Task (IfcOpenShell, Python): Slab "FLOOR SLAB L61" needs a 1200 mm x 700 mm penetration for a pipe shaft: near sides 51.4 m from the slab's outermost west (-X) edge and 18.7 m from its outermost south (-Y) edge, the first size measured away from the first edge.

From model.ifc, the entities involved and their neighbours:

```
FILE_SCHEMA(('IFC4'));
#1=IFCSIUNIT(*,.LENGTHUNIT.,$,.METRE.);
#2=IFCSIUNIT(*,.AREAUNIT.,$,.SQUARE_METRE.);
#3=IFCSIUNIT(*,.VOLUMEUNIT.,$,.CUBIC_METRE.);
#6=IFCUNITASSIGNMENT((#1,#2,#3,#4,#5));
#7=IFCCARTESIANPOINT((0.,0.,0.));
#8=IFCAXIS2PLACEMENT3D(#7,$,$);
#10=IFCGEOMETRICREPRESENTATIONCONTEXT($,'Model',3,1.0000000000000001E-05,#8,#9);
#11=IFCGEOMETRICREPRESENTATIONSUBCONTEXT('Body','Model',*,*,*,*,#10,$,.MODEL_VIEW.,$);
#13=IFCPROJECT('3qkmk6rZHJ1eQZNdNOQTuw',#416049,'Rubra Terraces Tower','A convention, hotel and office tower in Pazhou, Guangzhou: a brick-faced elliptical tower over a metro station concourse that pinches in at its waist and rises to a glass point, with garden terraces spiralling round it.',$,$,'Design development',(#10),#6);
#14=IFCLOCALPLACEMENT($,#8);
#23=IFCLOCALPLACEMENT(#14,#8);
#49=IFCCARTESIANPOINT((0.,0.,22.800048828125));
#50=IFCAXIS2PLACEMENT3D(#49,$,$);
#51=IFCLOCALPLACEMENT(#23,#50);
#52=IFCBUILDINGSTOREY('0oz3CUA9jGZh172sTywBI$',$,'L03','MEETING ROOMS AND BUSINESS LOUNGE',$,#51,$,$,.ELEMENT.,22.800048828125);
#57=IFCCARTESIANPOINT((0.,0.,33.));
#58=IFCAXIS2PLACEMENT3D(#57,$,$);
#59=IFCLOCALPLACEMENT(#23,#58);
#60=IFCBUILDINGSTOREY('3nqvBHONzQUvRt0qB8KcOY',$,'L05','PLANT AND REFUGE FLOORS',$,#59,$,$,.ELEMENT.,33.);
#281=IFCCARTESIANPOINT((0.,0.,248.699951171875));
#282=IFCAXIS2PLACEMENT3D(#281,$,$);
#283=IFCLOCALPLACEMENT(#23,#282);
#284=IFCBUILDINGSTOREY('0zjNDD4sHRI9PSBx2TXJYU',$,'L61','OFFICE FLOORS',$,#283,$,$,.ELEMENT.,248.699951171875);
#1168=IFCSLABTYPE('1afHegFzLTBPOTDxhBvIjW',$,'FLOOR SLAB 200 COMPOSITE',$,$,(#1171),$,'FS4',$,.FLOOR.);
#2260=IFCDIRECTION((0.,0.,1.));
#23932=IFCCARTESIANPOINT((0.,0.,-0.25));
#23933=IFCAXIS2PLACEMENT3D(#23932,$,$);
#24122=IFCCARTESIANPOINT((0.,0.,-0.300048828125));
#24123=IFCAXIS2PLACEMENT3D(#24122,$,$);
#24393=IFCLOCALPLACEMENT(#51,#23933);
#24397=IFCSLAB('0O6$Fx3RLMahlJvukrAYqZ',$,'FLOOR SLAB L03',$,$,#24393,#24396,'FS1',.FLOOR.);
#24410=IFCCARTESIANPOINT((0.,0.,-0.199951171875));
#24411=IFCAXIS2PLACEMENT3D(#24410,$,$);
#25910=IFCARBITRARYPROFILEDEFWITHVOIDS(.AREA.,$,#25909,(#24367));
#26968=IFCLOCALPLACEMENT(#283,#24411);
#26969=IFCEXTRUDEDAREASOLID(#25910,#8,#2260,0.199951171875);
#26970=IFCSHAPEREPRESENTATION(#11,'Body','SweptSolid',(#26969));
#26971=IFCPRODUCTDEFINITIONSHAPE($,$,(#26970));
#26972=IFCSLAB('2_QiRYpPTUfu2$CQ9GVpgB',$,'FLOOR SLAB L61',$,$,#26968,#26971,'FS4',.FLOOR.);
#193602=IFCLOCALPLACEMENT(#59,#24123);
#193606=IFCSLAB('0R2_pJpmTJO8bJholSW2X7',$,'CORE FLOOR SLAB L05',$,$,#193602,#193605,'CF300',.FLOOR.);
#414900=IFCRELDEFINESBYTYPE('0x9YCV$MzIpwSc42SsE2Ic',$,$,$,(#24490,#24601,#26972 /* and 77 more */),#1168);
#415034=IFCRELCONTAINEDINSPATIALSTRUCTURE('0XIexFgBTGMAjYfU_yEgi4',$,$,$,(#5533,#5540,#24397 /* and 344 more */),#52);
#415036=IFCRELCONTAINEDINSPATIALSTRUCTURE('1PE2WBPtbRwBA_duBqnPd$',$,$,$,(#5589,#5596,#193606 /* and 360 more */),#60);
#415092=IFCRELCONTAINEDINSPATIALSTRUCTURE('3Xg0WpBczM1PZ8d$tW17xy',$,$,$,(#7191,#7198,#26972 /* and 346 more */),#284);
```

```python
import numpy as np
import ifcopenshell
import ifcopenshell.api.feature
import ifcopenshell.api.geometry
import ifcopenshell.api.root
import ifcopenshell.geom
import ifcopenshell.util.placement
import ifcopenshell.util.representation
import ifcopenshell.util.shape
import ifcopenshell.util.unit

model = ifcopenshell.open("model.ifc")
unit_scale = ifcopenshell.util.unit.calculate_unit_scale(model)
settings = ifcopenshell.geom.settings()


def volume(element):
    """Net volume in cubic metres, openings subtracted."""
    shape = ifcopenshell.geom.create_shape(settings, element)
    return ifcopenshell.util.shape.get_volume(shape.geometry)


slab = model.by_guid("2_QiRYpPTUfu2$CQ9GVpgB")
before = volume(slab)

# Extent in the slab's own axes, in metres. The edges named are its -X and -Y sides.
slab_shape = ifcopenshell.geom.create_shape(settings, slab)
vertices = ifcopenshell.util.shape.get_vertices(slab_shape.geometry)
x_min, y_min, bottom = vertices.min(axis=0)
top = vertices[:, 2].max()

opening = ifcopenshell.api.root.create_entity(model, ifc_class="IfcOpeningElement", name="Pipe shaft opening", predefined_type="OPENING")
context = ifcopenshell.util.representation.get_context(model, "Model", "Body", "MODEL_VIEW")
width, depth = 1.2, 0.7
outline = [(0.0, 0.0), (width, 0.0), (width, depth), (0.0, depth), (0.0, 0.0)]
# Overshoot both faces by 50 mm so the cut is clean.
shape = ifcopenshell.api.geometry.add_slab_representation(
    model, context=context, depth=top - bottom + 0.1, polyline=outline
)
ifcopenshell.api.geometry.assign_representation(model, product=opening, representation=shape)

matrix = ifcopenshell.util.placement.get_local_placement(slab.ObjectPlacement)
matrix[:, 3] = matrix @ np.append(np.array([x_min + 51.4, y_min + 18.7, bottom - 0.05]) / unit_scale, 1.0)
ifcopenshell.api.geometry.edit_object_placement(model, product=opening, matrix=matrix, is_si=False)
ifcopenshell.api.feature.add_feature(model, feature=opening, element=slab)

after = volume(slab)

print(f"slab volume {before:.3f} -> {after:.3f} m3")

model.write("model_v2.ifc")
```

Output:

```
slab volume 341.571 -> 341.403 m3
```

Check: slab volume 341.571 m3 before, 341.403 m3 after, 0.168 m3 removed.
